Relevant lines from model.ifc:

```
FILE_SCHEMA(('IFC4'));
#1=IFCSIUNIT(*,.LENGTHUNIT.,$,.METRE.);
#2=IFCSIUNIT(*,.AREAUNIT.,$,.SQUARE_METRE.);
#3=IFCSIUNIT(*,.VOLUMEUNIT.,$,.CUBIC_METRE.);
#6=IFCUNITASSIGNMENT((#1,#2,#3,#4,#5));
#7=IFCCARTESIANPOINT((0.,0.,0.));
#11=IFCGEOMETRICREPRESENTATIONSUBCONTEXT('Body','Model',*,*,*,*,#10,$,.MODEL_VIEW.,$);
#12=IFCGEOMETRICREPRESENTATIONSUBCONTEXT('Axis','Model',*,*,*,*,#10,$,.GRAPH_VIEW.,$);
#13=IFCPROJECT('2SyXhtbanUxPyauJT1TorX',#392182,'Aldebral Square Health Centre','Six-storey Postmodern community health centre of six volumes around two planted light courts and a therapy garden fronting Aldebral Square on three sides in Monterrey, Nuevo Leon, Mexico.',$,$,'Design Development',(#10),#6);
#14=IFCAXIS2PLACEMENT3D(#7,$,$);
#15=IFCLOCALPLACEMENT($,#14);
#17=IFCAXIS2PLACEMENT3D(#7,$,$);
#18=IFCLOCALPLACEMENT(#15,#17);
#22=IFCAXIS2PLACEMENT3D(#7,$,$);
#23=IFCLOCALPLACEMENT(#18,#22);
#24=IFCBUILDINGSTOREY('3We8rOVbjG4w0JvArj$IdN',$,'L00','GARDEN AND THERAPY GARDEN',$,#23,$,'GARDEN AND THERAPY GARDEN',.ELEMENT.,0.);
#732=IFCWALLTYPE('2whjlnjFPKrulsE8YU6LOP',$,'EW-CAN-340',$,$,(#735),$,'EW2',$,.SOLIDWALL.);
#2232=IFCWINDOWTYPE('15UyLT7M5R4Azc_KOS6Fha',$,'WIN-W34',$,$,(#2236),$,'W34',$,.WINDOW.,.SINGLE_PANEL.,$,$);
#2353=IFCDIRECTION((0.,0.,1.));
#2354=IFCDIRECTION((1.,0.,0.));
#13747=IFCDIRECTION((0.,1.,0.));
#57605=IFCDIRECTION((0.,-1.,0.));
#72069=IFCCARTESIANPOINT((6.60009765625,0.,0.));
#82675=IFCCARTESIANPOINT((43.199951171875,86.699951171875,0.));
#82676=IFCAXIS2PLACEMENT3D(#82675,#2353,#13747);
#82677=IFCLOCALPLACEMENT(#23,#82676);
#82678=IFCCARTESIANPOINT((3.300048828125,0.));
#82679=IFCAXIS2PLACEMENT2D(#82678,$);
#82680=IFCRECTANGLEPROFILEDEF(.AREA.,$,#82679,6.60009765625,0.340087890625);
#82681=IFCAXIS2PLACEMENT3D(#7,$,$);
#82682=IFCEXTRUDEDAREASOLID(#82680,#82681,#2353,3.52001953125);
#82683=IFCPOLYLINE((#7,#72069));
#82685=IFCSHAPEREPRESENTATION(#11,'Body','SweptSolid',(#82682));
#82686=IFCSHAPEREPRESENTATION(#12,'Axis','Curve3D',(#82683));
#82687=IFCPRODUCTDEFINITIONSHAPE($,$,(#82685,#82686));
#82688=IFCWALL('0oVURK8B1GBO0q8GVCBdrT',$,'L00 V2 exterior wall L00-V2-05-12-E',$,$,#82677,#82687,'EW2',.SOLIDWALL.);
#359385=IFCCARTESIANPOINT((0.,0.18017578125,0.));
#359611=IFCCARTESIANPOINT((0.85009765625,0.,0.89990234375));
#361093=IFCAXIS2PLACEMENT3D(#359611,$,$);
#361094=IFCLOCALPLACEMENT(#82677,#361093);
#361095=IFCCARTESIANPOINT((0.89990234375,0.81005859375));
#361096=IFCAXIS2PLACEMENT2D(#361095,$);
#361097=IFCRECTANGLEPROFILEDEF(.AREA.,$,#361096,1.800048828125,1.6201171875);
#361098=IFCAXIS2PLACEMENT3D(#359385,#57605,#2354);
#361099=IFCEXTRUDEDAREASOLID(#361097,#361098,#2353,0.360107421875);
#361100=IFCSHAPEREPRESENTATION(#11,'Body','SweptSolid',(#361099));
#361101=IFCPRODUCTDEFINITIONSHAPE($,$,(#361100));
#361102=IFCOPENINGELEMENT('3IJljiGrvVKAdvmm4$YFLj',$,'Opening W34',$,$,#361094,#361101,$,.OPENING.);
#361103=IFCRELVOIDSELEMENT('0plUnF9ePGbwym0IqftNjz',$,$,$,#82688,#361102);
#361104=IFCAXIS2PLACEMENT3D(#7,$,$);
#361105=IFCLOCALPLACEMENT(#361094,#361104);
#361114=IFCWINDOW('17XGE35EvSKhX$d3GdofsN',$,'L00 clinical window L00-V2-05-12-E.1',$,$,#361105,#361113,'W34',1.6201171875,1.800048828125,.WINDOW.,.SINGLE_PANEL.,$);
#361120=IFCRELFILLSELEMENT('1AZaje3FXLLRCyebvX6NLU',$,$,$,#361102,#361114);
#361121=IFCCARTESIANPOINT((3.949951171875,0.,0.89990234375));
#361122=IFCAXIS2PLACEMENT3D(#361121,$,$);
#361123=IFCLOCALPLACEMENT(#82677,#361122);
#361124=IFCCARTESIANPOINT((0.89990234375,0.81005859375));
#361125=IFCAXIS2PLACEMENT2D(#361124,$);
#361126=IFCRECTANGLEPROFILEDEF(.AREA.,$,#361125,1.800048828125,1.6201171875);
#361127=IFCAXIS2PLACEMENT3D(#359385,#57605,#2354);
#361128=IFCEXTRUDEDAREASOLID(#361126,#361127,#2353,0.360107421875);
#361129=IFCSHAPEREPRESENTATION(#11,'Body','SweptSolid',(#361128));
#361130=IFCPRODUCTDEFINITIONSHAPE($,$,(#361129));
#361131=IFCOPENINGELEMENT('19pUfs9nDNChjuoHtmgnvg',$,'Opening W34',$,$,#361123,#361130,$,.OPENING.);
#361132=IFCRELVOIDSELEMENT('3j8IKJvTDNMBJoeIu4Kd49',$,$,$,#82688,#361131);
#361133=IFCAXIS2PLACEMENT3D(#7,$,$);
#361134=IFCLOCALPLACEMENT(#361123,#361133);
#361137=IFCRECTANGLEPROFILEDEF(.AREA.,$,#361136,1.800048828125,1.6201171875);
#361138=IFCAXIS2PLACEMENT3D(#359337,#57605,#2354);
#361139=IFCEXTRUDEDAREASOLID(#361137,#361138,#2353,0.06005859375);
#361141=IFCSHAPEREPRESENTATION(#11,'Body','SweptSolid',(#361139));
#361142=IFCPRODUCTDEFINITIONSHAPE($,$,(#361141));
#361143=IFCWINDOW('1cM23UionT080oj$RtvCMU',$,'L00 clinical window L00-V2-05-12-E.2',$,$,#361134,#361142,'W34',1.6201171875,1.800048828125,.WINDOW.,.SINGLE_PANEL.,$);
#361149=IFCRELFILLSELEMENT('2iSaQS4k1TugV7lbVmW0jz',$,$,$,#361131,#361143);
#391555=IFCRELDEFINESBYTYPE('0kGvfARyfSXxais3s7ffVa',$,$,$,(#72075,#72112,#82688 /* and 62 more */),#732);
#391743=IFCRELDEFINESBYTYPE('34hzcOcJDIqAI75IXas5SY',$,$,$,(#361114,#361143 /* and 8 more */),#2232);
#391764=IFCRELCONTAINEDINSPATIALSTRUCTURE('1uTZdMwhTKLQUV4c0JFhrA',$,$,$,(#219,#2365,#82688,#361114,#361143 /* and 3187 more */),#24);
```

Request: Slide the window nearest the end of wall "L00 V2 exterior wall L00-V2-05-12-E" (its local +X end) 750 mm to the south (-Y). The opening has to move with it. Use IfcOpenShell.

```python
import ifcopenshell
import ifcopenshell.api.geometry
import ifcopenshell.util.placement

model = ifcopenshell.open("model.ifc")

window = model.by_guid("1cM23UionT080oj$RtvCMU")
opening = window.FillsVoids[0].RelatingOpeningElement
wall = opening.VoidsElements[0].RelatingBuildingElement

wall_matrix = ifcopenshell.util.placement.get_local_placement(wall.ObjectPlacement)
shift = wall_matrix[:3, 0] * -0.75
before = ifcopenshell.util.placement.get_local_placement(window.ObjectPlacement)[:3, 3].copy()

# The window is placed relative to its opening, so it follows when the opening moves.
matrix = ifcopenshell.util.placement.get_local_placement(opening.ObjectPlacement)
matrix[:3, 3] += shift
ifcopenshell.api.geometry.edit_object_placement(
    model, product=opening, matrix=matrix, is_si=False, should_transform_children=True
)

after = ifcopenshell.util.placement.get_local_placement(window.ObjectPlacement)[:3, 3]
print("window moved by", (after - before).round(3) + 0.0)

model.write("model_rev.ifc")
```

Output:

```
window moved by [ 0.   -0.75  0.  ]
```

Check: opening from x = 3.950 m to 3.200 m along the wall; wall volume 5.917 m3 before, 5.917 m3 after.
